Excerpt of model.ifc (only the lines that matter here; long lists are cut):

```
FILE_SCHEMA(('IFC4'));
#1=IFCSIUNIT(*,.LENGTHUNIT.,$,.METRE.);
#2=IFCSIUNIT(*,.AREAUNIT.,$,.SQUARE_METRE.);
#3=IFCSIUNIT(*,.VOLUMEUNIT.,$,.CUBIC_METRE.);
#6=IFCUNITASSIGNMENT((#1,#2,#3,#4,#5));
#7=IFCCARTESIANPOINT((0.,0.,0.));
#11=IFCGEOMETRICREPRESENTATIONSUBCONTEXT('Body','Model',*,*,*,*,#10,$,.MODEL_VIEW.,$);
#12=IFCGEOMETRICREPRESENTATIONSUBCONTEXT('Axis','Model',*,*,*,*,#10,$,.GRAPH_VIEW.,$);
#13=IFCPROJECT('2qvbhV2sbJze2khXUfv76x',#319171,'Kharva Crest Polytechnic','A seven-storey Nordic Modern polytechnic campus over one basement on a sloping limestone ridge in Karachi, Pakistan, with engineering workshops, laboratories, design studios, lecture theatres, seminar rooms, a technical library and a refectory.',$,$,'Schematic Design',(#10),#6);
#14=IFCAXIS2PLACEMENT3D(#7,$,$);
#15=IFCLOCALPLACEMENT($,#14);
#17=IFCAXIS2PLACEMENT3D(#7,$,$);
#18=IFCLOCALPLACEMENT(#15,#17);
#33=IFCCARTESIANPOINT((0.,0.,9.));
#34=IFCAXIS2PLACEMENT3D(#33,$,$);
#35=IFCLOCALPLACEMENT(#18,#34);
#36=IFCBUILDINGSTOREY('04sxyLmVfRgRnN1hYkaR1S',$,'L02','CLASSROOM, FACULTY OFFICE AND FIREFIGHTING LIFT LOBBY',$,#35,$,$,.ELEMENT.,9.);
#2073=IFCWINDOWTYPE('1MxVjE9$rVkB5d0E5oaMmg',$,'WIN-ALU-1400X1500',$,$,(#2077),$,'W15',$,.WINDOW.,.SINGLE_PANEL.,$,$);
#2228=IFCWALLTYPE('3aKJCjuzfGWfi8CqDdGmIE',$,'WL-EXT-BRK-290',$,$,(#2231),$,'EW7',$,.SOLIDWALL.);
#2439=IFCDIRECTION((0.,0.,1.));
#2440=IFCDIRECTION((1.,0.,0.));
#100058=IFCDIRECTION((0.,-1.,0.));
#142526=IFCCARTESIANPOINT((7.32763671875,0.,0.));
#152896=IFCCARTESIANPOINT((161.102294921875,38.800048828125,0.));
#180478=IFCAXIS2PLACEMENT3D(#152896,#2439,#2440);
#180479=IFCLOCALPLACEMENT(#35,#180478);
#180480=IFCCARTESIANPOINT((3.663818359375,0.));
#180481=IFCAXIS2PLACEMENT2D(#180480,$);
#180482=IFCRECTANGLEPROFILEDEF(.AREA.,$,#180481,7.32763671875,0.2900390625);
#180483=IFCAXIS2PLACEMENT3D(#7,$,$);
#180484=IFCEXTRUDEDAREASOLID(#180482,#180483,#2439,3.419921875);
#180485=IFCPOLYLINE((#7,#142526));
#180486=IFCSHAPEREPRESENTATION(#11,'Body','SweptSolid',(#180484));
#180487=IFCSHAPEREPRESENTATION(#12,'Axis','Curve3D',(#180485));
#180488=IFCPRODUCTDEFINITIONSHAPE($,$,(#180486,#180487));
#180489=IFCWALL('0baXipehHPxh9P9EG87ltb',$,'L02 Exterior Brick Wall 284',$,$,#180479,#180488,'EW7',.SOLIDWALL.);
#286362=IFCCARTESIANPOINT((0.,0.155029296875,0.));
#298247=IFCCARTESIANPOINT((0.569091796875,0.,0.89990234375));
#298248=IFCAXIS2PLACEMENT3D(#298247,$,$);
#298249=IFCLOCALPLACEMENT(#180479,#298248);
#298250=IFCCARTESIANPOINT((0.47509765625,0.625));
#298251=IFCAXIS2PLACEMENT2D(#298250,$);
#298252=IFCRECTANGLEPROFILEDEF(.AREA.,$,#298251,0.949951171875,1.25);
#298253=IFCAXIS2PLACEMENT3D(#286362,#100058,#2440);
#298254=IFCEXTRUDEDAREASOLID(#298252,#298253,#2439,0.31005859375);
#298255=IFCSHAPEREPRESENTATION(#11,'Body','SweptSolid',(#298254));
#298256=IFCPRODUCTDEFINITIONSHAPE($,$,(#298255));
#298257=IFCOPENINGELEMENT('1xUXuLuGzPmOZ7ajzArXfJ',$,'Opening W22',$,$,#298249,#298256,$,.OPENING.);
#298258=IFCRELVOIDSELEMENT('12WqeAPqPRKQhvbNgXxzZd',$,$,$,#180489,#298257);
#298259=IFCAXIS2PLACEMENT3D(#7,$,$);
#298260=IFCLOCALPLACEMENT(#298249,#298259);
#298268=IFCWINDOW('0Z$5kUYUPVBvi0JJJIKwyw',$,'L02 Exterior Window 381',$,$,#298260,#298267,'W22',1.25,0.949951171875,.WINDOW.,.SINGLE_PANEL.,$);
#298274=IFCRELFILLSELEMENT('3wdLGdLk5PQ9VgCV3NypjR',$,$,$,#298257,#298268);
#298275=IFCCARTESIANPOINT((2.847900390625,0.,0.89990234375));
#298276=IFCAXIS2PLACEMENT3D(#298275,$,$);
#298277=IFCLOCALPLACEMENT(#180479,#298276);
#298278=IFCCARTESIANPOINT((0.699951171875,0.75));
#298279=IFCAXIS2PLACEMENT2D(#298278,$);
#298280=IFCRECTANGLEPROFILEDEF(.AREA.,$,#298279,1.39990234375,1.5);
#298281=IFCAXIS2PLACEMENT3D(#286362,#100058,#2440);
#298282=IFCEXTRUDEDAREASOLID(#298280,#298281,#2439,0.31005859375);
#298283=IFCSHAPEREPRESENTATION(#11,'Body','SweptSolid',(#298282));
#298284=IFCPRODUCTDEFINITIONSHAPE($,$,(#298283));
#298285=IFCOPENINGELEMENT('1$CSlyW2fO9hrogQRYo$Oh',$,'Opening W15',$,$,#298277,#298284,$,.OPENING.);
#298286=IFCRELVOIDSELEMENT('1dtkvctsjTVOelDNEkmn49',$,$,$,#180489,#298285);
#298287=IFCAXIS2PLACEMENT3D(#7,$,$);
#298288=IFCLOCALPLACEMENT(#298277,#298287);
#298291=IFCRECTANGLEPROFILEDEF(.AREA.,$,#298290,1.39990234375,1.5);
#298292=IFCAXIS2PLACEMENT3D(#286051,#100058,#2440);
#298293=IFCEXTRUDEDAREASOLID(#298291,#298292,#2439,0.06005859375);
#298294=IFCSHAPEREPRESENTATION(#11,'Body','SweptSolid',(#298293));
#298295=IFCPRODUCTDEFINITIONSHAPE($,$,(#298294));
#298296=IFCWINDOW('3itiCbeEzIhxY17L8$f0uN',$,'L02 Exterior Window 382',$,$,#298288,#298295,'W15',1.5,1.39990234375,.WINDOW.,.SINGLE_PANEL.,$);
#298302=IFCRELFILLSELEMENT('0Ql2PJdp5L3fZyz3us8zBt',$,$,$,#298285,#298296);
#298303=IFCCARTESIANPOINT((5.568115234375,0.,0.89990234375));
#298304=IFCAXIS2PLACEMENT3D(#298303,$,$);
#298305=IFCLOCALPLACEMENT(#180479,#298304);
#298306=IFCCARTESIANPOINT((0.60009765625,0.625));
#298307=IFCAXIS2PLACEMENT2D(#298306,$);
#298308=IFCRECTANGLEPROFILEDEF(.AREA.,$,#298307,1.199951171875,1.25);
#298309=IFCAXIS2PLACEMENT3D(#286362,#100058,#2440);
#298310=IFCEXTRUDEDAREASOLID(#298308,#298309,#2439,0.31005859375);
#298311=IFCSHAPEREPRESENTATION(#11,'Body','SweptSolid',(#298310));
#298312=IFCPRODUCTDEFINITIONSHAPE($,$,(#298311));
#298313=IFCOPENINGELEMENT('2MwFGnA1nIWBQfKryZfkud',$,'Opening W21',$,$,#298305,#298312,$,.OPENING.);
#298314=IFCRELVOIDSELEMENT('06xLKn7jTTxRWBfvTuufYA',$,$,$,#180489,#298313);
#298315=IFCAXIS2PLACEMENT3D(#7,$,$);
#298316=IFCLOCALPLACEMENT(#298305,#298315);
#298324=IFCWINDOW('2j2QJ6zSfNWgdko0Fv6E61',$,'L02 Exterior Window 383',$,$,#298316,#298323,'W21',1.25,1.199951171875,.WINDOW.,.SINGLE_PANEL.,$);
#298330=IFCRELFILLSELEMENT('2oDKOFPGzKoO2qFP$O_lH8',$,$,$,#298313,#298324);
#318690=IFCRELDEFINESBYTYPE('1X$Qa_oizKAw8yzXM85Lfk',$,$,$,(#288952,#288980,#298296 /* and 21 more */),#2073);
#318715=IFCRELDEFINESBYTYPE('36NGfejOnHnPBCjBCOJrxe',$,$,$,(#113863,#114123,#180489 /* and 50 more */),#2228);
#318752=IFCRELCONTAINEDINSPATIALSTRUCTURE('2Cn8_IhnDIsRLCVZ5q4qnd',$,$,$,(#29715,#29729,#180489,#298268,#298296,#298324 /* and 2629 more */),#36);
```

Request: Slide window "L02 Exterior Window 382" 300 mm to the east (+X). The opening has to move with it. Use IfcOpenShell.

```python
import ifcopenshell
import ifcopenshell.api.geometry
import ifcopenshell.util.placement
import ifcopenshell.util.unit

model = ifcopenshell.open("model.ifc")
unit_scale = ifcopenshell.util.unit.calculate_unit_scale(model)

window = model.by_id(298296)
opening = window.FillsVoids[0].RelatingOpeningElement
wall = opening.VoidsElements[0].RelatingBuildingElement

wall_matrix = ifcopenshell.util.placement.get_local_placement(wall.ObjectPlacement)
shift = wall_matrix[:3, 0] * 0.3 / unit_scale
before = ifcopenshell.util.placement.get_local_placement(window.ObjectPlacement)[:3, 3].copy()

# The window is placed relative to its opening, so it follows when the opening moves.
matrix = ifcopenshell.util.placement.get_local_placement(opening.ObjectPlacement)
matrix[:3, 3] += shift
ifcopenshell.api.geometry.edit_object_placement(
    model, product=opening, matrix=matrix, is_si=False, should_transform_children=True
)

after = ifcopenshell.util.placement.get_local_placement(window.ObjectPlacement)[:3, 3]
print("window moved by", (after - before).round(3) + 0.0)

model.write("model_updated.ifc")
```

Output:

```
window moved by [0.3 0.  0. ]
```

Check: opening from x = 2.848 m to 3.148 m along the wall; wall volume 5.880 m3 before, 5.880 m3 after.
